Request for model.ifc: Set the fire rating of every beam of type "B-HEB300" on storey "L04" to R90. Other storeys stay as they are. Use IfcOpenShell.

First a look at what the model holds.

```python
import ifcopenshell
import ifcopenshell.util.element

model = ifcopenshell.open("model.ifc")
print(model.schema)
storey = next(s for s in model.by_type("IfcBuildingStorey") if s.Name == "L04")
beams = [e for e in ifcopenshell.util.element.get_decomposition(storey) if e.is_a("IfcBeam")]
seen = {}
for e in beams:
    element_type = ifcopenshell.util.element.get_type(e)
    key = (element_type.Name if element_type != e and element_type else None, ifcopenshell.util.element.get_pset(e, "Pset_BeamCommon", "FireRating"))
    seen[key] = seen.get(key, 0) + 1
for (name, value), count in sorted(seen.items(), key=str):
    print(count, "x", name, "|", value)
```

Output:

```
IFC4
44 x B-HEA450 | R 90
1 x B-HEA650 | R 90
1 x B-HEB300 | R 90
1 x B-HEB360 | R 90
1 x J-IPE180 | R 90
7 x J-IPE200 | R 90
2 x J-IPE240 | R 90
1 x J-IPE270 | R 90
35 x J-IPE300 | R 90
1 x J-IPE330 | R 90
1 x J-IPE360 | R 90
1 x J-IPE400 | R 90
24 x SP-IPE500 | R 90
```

```python
import ifcopenshell
import ifcopenshell.api.pset
import ifcopenshell.util.element

model = ifcopenshell.open("model.ifc")

storey = next(s for s in model.by_type("IfcBuildingStorey") if s.Name == "L04")
beams = [e for e in ifcopenshell.util.element.get_decomposition(storey) if e.is_a("IfcBeam")]

count = 0
for e in beams:
    element_type = ifcopenshell.util.element.get_type(e)
    if element_type in (None, e) or element_type.Name != "B-HEB300":
        continue
    # add_pset returns the element's existing set when there is one.
    pset = ifcopenshell.api.pset.add_pset(model, product=e, name="Pset_BeamCommon")
    ifcopenshell.api.pset.edit_pset(model, pset=pset, properties={"FireRating": "R90"})
    count += 1

print(count, "beams updated")

model.write("model-out.ifc")
```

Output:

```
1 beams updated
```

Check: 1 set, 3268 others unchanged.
